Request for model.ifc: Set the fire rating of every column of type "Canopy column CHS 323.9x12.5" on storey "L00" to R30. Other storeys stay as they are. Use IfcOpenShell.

First a look at what the model holds.

```python
import ifcopenshell
import ifcopenshell.util.element

model = ifcopenshell.open("model.ifc")
print(model.schema)
storey = next(s for s in model.by_type("IfcBuildingStorey") if s.Name == "L00")
columns = [e for e in ifcopenshell.util.element.get_decomposition(storey) if e.is_a("IfcColumn")]
seen = {}
for e in columns:
    element_type = ifcopenshell.util.element.get_type(e)
    key = (element_type.Name if element_type != e and element_type else None, ifcopenshell.util.element.get_pset(e, "Pset_ColumnCommon", "FireRating"))
    seen[key] = seen.get(key, 0) + 1
for (name, value), count in sorted(seen.items(), key=str):
    print(count, "x", name, "|", value)
```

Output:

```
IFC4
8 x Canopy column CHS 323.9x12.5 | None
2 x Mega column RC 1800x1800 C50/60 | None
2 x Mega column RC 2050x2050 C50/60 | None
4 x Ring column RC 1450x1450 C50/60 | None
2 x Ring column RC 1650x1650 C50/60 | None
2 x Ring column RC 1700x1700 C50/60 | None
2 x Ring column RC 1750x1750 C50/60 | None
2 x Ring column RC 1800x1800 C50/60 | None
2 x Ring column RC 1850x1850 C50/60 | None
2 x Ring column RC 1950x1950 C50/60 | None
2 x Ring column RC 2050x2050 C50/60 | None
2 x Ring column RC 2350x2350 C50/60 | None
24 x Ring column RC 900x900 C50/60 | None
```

```python
import ifcopenshell
import ifcopenshell.api.pset
import ifcopenshell.util.element

model = ifcopenshell.open("model.ifc")

storey = next(s for s in model.by_type("IfcBuildingStorey") if s.Name == "L00")
columns = [e for e in ifcopenshell.util.element.get_decomposition(storey) if e.is_a("IfcColumn")]

count = 0
for e in columns:
    element_type = ifcopenshell.util.element.get_type(e)
    if element_type in (None, e) or element_type.Name != "Canopy column CHS 323.9x12.5":
        continue
    found = ifcopenshell.util.element.get_pset(e, "Pset_ColumnCommon", should_inherit=False)
    if found:
        pset = model.by_id(found["id"])
        if len(ifcopenshell.util.element.get_elements_by_pset(pset)) > 1:
            pset = ifcopenshell.api.pset.unshare_pset(model, products=[e], pset=pset)[0]
    else:
        pset = ifcopenshell.api.pset.add_pset(model, product=e, name="Pset_ColumnCommon")
    ifcopenshell.api.pset.edit_pset(model, pset=pset, properties={"FireRating": "R30"})
    count += 1

print(count, "columns updated")

model.write("model-out.ifc")
```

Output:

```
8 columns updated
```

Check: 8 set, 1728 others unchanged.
